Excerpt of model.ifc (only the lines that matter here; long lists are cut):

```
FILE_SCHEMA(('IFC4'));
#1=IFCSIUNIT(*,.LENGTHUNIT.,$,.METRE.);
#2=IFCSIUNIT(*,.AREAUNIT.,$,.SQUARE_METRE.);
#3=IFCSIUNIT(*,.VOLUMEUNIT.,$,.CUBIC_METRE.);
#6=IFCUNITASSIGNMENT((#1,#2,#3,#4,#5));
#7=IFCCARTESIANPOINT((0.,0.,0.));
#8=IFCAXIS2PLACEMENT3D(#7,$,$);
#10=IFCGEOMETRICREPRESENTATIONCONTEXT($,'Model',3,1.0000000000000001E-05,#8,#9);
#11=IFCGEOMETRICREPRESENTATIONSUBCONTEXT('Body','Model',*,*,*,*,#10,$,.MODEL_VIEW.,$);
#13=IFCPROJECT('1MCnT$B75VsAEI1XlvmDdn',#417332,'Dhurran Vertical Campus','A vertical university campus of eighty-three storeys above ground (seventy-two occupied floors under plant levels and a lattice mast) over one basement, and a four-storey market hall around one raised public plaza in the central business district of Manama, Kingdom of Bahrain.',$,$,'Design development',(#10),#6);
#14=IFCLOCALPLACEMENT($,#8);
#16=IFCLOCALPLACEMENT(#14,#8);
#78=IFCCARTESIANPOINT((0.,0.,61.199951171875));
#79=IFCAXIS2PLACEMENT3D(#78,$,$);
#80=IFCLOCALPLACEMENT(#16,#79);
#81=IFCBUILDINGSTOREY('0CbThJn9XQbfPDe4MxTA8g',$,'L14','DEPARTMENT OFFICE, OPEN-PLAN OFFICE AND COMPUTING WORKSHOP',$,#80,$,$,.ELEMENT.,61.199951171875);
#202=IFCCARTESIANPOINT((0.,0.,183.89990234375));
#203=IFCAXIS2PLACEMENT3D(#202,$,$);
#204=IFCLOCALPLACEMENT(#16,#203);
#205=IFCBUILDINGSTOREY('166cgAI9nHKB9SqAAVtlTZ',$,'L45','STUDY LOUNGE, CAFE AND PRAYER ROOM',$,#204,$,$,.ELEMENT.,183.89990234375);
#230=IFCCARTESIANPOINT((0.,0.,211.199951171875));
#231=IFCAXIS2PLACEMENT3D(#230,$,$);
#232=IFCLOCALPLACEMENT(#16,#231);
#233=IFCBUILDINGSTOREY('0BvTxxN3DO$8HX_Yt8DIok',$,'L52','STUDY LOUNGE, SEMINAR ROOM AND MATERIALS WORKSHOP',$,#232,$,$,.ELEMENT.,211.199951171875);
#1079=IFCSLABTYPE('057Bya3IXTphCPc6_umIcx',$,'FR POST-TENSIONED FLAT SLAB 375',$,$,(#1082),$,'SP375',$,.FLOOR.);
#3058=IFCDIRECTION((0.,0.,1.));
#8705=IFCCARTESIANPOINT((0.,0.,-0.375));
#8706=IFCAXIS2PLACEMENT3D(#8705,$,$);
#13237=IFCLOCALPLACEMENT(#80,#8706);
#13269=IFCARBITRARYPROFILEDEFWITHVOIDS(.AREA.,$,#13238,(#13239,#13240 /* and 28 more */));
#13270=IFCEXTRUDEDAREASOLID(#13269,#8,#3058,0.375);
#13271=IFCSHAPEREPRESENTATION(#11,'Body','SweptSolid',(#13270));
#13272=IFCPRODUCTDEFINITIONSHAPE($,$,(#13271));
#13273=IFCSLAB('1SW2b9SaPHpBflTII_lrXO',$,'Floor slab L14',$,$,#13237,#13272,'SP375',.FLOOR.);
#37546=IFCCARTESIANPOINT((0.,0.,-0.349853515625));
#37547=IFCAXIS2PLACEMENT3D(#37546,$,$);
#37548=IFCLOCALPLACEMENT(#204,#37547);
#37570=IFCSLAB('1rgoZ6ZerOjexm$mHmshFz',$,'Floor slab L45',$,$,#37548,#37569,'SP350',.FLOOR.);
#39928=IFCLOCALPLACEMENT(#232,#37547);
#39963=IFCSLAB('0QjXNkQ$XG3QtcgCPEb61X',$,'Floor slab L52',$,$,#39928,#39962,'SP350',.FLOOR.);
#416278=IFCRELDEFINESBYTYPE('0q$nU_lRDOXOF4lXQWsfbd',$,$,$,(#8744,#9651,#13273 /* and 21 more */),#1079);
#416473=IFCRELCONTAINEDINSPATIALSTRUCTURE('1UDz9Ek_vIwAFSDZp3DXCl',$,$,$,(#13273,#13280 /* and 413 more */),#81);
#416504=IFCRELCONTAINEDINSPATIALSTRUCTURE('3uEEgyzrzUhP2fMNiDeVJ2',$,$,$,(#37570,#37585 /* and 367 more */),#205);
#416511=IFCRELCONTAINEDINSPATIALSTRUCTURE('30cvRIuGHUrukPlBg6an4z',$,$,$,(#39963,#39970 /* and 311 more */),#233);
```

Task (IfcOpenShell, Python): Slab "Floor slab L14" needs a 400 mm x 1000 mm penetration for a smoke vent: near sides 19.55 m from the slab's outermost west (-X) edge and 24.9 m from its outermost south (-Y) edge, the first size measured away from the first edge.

```python
import numpy as np
import ifcopenshell
import ifcopenshell.api.feature
import ifcopenshell.api.geometry
import ifcopenshell.api.root
import ifcopenshell.geom
import ifcopenshell.util.placement
import ifcopenshell.util.representation
import ifcopenshell.util.shape
import ifcopenshell.util.unit

model = ifcopenshell.open("model.ifc")
unit_scale = ifcopenshell.util.unit.calculate_unit_scale(model)
settings = ifcopenshell.geom.settings()


def volume(element):
    """Net volume in cubic metres, openings subtracted."""
    shape = ifcopenshell.geom.create_shape(settings, element)
    return ifcopenshell.util.shape.get_volume(shape.geometry)


slab = model.by_guid("1SW2b9SaPHpBflTII_lrXO")
before = volume(slab)

# Extent in the slab's own axes, in metres. The edges named are its -X and -Y sides.
slab_shape = ifcopenshell.geom.create_shape(settings, slab)
vertices = ifcopenshell.util.shape.get_vertices(slab_shape.geometry)
x_min, y_min, bottom = vertices.min(axis=0)
top = vertices[:, 2].max()

opening = ifcopenshell.api.root.create_entity(model, ifc_class="IfcOpeningElement", name="Smoke vent opening", predefined_type="OPENING")
context = ifcopenshell.util.representation.get_context(model, "Model", "Body", "MODEL_VIEW")
width, depth = 0.4, 1
outline = [(0.0, 0.0), (width, 0.0), (width, depth), (0.0, depth), (0.0, 0.0)]
# Overshoot both faces by 50 mm so the cut is clean.
shape = ifcopenshell.api.geometry.add_slab_representation(
    model, context=context, depth=top - bottom + 0.1, polyline=outline
)
ifcopenshell.api.geometry.assign_representation(model, product=opening, representation=shape)

matrix = ifcopenshell.util.placement.get_local_placement(slab.ObjectPlacement)
matrix[:, 3] = matrix @ np.append(np.array([x_min + 19.55, y_min + 24.9, bottom - 0.05]) / unit_scale, 1.0)
ifcopenshell.api.geometry.edit_object_placement(model, product=opening, matrix=matrix, is_si=False)
ifcopenshell.api.feature.add_feature(model, feature=opening, element=slab)

after = volume(slab)

print(f"slab volume {before:.3f} -> {after:.3f} m3")

model.write("model_updated.ifc")
```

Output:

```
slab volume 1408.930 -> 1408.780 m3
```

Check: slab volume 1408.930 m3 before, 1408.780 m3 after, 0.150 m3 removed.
